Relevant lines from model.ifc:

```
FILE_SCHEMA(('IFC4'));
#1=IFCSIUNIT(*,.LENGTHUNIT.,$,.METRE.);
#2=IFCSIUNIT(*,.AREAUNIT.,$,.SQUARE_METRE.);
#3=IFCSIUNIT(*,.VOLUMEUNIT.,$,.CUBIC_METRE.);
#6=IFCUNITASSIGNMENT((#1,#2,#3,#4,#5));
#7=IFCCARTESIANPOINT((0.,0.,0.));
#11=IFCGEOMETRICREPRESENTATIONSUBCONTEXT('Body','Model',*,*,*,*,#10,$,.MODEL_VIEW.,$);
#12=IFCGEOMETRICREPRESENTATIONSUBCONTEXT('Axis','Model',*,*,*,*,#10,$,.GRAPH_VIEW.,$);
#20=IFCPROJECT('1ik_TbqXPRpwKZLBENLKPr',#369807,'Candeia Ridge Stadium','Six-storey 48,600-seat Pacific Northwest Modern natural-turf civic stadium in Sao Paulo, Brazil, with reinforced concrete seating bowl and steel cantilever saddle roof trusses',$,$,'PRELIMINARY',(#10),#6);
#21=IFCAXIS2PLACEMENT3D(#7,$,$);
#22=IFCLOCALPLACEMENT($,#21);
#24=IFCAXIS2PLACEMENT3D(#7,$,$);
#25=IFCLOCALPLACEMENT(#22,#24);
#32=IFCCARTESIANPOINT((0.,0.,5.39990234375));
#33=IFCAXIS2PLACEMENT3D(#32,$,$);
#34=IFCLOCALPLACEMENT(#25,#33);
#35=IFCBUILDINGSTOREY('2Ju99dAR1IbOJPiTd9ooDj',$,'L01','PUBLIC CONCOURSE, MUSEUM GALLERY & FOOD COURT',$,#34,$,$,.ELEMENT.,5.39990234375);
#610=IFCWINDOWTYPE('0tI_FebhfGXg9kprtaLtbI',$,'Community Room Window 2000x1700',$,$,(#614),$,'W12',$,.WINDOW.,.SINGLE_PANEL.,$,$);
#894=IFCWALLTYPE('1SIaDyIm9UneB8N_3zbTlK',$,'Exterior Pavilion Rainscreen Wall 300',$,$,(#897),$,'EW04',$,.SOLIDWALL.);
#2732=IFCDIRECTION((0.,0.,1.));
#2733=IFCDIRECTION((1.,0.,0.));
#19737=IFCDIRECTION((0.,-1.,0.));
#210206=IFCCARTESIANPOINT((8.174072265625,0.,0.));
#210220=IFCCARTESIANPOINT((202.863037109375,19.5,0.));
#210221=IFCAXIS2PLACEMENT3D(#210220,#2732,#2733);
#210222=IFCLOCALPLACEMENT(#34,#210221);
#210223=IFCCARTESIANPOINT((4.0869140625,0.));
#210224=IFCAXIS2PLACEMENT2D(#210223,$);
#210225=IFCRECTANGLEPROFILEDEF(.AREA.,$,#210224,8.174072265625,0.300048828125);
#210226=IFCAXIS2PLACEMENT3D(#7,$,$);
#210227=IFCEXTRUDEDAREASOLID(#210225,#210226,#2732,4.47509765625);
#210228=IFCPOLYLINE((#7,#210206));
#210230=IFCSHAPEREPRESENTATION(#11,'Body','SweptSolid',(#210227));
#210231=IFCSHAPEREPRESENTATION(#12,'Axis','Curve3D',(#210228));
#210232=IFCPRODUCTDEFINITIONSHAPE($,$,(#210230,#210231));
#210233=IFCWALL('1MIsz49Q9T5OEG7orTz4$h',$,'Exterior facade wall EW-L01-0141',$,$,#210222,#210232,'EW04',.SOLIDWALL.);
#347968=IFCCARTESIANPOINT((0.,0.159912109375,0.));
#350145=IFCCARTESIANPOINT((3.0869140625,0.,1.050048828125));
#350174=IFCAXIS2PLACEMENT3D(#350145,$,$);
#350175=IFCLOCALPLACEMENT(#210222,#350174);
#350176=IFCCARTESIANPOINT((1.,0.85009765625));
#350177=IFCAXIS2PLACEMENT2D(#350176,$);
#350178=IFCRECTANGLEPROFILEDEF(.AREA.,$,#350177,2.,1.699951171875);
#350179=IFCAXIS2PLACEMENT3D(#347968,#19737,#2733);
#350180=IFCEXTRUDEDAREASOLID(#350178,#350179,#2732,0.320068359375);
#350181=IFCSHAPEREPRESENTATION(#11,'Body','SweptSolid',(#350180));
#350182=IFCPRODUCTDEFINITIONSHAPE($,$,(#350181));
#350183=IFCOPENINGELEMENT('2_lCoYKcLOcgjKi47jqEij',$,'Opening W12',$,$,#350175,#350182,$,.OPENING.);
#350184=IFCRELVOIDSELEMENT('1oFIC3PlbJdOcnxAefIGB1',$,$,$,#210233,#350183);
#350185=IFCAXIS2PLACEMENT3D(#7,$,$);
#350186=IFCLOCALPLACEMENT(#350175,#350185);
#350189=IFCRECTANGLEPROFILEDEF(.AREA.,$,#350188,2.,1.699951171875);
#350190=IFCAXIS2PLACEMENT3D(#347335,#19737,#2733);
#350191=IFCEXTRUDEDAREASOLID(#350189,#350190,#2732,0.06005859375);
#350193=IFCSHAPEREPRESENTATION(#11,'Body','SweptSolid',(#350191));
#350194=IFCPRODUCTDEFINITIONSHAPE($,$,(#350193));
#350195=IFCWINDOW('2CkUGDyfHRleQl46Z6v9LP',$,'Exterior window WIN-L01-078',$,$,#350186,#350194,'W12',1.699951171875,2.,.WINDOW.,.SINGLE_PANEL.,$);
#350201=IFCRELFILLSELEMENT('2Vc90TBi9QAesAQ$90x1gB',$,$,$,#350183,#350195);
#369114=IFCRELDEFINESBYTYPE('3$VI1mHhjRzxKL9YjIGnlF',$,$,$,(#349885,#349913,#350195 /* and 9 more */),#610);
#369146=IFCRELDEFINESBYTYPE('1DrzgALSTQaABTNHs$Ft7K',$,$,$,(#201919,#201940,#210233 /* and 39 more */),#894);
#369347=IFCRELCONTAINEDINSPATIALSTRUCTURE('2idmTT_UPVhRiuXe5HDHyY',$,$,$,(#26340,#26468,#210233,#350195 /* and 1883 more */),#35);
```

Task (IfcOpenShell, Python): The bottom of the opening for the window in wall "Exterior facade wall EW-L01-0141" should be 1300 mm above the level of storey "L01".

```python
import numpy as np
import ifcopenshell
import ifcopenshell.api.geometry
import ifcopenshell.geom
import ifcopenshell.util.element
import ifcopenshell.util.placement
import ifcopenshell.util.shape
import ifcopenshell.util.unit

model = ifcopenshell.open("model.ifc")
unit_scale = ifcopenshell.util.unit.calculate_unit_scale(model)

window = model.by_guid("2CkUGDyfHRleQl46Z6v9LP")
opening = window.FillsVoids[0].RelatingOpeningElement
storey = ifcopenshell.util.element.get_container(window, ifc_class="IfcBuildingStorey")
level = ifcopenshell.util.placement.get_local_placement(storey.ObjectPlacement)[2, 3]

# The opening's origin need not be at the sill, so measure its lowest point.
shape = ifcopenshell.geom.create_shape(ifcopenshell.geom.settings(), opening)
bottom = ifcopenshell.util.shape.get_shape_bottom_elevation(shape, shape.geometry) / unit_scale
dz = level + 1.3 - bottom

shift = np.array([0.0, 0.0, dz])
# The window is placed relative to its opening, so it follows when the opening moves.
matrix = ifcopenshell.util.placement.get_local_placement(opening.ObjectPlacement)
matrix[:3, 3] += shift
ifcopenshell.api.geometry.edit_object_placement(
    model, product=opening, matrix=matrix, is_si=False, should_transform_children=True
)

print(f"moved by {dz * unit_scale:+.3f} m")

model.write("model_rev.ifc")
```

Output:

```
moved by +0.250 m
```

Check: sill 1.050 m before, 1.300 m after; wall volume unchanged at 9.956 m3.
